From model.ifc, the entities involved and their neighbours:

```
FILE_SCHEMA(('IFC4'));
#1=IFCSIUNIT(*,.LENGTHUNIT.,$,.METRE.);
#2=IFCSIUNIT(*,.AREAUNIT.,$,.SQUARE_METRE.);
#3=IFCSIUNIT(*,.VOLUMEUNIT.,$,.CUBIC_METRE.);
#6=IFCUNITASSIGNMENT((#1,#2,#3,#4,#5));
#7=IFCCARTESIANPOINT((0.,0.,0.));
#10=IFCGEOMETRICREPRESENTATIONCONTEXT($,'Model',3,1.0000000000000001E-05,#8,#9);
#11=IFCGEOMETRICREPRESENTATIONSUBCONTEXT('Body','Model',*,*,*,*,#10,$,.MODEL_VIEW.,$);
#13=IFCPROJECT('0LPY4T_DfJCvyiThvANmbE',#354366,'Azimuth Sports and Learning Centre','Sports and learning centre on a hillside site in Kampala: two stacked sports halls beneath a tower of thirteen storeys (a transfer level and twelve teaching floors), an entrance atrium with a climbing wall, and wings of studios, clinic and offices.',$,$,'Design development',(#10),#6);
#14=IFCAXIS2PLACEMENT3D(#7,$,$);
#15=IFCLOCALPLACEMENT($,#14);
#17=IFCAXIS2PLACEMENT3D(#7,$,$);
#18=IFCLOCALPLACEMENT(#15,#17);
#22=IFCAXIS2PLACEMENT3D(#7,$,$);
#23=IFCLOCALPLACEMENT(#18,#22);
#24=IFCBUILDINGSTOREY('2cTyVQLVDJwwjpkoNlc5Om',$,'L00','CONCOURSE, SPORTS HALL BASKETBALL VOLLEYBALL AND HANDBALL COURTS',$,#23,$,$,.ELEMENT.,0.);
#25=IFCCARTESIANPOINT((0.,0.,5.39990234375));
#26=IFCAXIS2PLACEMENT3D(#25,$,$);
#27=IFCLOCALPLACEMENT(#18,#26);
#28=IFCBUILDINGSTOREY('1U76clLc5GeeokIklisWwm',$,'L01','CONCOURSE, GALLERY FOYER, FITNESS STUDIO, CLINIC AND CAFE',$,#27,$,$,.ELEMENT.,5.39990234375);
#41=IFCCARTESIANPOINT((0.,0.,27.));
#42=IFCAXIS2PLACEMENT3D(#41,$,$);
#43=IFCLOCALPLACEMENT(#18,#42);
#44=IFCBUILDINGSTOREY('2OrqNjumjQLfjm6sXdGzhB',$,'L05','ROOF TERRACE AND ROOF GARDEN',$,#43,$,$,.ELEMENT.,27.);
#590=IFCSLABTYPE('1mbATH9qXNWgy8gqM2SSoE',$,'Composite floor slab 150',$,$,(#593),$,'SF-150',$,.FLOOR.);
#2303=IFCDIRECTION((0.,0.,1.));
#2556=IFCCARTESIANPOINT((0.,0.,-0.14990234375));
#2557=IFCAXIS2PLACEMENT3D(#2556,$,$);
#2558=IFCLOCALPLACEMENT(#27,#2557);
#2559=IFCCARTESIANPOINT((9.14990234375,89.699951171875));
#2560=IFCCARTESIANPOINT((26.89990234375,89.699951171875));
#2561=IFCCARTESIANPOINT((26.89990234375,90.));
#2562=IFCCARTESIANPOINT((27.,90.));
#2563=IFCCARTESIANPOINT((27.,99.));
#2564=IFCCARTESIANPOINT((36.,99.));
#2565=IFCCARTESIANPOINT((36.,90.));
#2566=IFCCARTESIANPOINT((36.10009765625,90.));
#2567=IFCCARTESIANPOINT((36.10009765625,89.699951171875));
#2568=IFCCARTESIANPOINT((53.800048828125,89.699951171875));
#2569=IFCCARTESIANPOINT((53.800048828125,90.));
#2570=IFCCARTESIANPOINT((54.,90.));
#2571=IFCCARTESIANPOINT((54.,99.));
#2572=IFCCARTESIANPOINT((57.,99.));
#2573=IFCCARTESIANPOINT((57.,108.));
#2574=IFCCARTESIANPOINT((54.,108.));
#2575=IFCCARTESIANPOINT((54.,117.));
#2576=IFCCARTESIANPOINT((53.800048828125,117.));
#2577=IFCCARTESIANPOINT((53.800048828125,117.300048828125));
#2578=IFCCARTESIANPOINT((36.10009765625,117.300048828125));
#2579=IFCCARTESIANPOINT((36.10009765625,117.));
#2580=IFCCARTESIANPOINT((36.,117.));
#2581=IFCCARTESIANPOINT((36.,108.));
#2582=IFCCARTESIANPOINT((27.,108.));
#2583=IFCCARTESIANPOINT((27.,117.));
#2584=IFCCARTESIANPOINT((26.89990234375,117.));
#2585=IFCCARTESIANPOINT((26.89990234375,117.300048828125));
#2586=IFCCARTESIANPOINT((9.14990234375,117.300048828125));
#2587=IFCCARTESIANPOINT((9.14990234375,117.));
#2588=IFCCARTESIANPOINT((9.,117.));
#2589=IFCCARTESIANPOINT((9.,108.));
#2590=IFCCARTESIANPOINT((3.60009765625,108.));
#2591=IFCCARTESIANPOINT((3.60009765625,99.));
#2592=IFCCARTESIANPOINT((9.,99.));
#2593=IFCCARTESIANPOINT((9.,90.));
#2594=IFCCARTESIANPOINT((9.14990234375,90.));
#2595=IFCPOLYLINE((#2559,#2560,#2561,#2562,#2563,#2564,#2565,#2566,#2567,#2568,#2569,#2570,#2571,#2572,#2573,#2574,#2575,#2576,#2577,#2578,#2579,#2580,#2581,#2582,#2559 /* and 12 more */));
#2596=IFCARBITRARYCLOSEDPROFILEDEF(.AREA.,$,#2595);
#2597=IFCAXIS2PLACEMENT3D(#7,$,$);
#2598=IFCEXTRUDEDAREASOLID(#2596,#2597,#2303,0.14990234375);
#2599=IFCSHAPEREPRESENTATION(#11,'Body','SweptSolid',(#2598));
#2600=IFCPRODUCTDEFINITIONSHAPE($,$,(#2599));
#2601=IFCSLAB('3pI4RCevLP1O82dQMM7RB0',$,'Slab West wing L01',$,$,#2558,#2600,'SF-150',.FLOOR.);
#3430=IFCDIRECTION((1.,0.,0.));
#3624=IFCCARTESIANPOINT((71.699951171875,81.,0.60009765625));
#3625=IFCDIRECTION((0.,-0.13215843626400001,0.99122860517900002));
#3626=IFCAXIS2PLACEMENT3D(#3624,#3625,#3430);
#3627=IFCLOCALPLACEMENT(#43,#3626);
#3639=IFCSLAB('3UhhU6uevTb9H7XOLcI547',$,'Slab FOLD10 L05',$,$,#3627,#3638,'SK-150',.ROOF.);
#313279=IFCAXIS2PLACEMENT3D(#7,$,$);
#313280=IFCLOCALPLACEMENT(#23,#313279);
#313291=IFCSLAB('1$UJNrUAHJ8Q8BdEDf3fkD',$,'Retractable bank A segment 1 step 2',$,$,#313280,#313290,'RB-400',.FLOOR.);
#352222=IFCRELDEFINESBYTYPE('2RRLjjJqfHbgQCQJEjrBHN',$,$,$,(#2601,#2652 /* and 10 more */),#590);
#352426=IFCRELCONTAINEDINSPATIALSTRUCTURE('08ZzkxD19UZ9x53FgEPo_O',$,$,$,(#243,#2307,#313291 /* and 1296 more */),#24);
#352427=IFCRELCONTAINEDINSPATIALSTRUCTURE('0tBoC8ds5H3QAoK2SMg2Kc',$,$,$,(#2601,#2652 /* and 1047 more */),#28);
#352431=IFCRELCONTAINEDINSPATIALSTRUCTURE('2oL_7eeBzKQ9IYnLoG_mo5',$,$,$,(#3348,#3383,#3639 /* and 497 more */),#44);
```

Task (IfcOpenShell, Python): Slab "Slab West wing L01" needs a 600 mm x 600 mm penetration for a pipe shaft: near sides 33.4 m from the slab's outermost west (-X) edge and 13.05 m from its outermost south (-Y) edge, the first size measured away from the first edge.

```python
import numpy as np
import ifcopenshell
import ifcopenshell.api.feature
import ifcopenshell.api.geometry
import ifcopenshell.api.root
import ifcopenshell.geom
import ifcopenshell.util.placement
import ifcopenshell.util.representation
import ifcopenshell.util.shape
import ifcopenshell.util.unit

model = ifcopenshell.open("model.ifc")
unit_scale = ifcopenshell.util.unit.calculate_unit_scale(model)
settings = ifcopenshell.geom.settings()


def volume(element):
    """Net volume in cubic metres, openings subtracted."""
    shape = ifcopenshell.geom.create_shape(settings, element)
    return ifcopenshell.util.shape.get_volume(shape.geometry)


slab = model.by_guid("3pI4RCevLP1O82dQMM7RB0")
before = volume(slab)

# Extent in the slab's own axes, in metres. The edges named are its -X and -Y sides.
slab_shape = ifcopenshell.geom.create_shape(settings, slab)
vertices = ifcopenshell.util.shape.get_vertices(slab_shape.geometry)
x_min, y_min, bottom = vertices.min(axis=0)
top = vertices[:, 2].max()

opening = ifcopenshell.api.root.create_entity(model, ifc_class="IfcOpeningElement", name="Pipe shaft opening", predefined_type="OPENING")
context = ifcopenshell.util.representation.get_context(model, "Model", "Body", "MODEL_VIEW")
width, depth = 0.6, 0.6
outline = [(0.0, 0.0), (width, 0.0), (width, depth), (0.0, depth), (0.0, 0.0)]
# Overshoot both faces by 50 mm so the cut is clean.
shape = ifcopenshell.api.geometry.add_slab_representation(
    model, context=context, depth=top - bottom + 0.1, polyline=outline
)
ifcopenshell.api.geometry.assign_representation(model, product=opening, representation=shape)

matrix = ifcopenshell.util.placement.get_local_placement(slab.ObjectPlacement)
matrix[:, 3] = matrix @ np.append(np.array([x_min + 33.4, y_min + 13.05, bottom - 0.05]) / unit_scale, 1.0)
ifcopenshell.api.geometry.edit_object_placement(model, product=opening, matrix=matrix, is_si=False)
ifcopenshell.api.feature.add_feature(model, feature=opening, element=slab)

after = volume(slab)

print(f"slab volume {before:.3f} -> {after:.3f} m3")

model.write("model_updated.ifc")
```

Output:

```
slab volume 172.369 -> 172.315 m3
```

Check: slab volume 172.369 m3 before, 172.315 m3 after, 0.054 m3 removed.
